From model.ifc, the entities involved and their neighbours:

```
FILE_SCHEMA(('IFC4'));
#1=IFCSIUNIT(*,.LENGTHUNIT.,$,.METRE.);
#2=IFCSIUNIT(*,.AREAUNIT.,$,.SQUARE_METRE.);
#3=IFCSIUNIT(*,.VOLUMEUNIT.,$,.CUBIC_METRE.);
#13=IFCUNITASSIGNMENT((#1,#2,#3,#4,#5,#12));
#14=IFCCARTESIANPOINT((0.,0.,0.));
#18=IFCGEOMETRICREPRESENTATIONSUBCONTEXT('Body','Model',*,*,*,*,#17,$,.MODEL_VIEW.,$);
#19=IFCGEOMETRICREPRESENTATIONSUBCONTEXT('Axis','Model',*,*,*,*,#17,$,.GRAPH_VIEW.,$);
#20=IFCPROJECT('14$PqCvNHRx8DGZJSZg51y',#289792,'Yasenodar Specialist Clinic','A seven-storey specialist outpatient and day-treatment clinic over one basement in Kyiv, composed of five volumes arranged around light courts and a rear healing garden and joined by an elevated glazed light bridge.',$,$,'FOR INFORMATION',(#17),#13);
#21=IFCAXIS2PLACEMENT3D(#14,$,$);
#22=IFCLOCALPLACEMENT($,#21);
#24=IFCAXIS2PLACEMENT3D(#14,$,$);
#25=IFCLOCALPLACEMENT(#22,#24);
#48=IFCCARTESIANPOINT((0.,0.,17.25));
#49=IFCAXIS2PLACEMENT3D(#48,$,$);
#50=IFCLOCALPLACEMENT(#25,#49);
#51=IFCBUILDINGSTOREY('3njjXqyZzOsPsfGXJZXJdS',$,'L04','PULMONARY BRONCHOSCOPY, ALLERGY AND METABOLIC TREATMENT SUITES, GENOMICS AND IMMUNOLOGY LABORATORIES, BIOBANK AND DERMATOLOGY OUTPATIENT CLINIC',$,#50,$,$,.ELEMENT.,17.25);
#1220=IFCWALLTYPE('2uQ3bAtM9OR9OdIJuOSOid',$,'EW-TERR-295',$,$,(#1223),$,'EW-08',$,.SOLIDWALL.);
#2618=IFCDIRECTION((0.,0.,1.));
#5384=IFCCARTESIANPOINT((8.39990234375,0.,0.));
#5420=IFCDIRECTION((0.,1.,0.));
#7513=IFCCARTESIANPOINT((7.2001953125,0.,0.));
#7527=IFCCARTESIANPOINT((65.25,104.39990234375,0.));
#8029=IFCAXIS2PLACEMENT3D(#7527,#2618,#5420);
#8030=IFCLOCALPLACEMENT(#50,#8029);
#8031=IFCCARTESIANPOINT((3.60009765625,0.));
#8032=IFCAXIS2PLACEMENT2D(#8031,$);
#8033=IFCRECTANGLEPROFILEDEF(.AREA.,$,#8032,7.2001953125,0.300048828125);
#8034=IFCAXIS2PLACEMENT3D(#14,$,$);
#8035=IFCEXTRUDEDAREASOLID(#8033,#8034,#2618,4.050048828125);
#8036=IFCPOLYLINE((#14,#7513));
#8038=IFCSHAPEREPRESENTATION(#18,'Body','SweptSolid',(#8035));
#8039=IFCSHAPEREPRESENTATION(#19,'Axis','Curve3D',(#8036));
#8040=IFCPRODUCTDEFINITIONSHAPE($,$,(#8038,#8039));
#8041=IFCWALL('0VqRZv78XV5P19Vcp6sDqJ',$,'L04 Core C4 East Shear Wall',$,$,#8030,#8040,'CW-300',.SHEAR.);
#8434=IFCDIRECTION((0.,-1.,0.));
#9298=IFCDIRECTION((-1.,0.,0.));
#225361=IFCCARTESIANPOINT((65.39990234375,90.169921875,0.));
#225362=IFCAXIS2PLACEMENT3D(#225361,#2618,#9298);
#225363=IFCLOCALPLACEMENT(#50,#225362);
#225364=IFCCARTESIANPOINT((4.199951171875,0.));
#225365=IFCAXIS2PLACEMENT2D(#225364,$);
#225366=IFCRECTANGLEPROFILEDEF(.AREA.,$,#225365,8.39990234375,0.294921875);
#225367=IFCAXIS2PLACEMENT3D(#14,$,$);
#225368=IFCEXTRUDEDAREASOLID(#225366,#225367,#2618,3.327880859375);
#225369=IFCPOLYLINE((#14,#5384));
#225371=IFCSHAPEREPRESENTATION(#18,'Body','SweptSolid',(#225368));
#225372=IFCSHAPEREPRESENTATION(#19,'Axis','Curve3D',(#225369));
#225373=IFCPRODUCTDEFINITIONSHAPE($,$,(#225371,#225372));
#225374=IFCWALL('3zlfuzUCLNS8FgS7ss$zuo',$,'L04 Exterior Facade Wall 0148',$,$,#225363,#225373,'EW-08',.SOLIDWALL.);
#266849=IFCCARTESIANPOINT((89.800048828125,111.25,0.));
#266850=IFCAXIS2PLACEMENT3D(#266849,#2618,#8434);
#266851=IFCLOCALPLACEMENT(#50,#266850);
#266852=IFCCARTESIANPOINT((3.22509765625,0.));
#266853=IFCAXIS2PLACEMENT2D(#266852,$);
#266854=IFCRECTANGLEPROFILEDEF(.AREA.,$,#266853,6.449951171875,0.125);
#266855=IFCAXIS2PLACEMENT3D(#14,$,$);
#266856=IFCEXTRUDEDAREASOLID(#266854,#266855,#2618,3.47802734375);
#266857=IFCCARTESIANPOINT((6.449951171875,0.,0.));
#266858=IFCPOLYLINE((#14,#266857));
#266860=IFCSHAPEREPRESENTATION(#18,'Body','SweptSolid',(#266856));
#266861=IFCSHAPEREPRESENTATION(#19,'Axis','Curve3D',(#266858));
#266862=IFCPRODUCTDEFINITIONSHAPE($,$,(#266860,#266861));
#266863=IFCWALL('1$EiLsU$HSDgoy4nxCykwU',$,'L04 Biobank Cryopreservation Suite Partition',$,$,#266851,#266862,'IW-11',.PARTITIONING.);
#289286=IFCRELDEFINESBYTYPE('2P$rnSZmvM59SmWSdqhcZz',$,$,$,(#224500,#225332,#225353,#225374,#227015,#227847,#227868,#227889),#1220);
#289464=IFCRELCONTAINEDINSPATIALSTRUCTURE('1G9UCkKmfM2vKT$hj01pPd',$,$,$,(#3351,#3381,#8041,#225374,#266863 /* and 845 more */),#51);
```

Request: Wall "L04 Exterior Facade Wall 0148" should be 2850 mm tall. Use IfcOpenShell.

```python
import ifcopenshell
import ifcopenshell.geom
import ifcopenshell.util.representation
import ifcopenshell.util.shape
import ifcopenshell.util.unit

model = ifcopenshell.open("model.ifc")
unit_scale = ifcopenshell.util.unit.calculate_unit_scale(model)
settings = ifcopenshell.geom.settings()


def volume(element):
    """Net volume in cubic metres, openings subtracted."""
    shape = ifcopenshell.geom.create_shape(settings, element)
    return ifcopenshell.util.shape.get_volume(shape.geometry)


wall = model.by_id(225374)
before = volume(wall)

body = ifcopenshell.util.representation.get_representation(wall, "Model", "Body")
solid = body.Items[0]
old_height = solid.Depth
solid.Depth = 2.85 / unit_scale
after = volume(wall)

print(f"height {old_height:g} -> {solid.Depth:g}, volume {before:.3f} -> {after:.3f} m3")

model.write("model-out.ifc")
```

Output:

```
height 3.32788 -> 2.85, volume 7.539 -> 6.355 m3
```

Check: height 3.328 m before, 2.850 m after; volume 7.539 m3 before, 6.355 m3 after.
